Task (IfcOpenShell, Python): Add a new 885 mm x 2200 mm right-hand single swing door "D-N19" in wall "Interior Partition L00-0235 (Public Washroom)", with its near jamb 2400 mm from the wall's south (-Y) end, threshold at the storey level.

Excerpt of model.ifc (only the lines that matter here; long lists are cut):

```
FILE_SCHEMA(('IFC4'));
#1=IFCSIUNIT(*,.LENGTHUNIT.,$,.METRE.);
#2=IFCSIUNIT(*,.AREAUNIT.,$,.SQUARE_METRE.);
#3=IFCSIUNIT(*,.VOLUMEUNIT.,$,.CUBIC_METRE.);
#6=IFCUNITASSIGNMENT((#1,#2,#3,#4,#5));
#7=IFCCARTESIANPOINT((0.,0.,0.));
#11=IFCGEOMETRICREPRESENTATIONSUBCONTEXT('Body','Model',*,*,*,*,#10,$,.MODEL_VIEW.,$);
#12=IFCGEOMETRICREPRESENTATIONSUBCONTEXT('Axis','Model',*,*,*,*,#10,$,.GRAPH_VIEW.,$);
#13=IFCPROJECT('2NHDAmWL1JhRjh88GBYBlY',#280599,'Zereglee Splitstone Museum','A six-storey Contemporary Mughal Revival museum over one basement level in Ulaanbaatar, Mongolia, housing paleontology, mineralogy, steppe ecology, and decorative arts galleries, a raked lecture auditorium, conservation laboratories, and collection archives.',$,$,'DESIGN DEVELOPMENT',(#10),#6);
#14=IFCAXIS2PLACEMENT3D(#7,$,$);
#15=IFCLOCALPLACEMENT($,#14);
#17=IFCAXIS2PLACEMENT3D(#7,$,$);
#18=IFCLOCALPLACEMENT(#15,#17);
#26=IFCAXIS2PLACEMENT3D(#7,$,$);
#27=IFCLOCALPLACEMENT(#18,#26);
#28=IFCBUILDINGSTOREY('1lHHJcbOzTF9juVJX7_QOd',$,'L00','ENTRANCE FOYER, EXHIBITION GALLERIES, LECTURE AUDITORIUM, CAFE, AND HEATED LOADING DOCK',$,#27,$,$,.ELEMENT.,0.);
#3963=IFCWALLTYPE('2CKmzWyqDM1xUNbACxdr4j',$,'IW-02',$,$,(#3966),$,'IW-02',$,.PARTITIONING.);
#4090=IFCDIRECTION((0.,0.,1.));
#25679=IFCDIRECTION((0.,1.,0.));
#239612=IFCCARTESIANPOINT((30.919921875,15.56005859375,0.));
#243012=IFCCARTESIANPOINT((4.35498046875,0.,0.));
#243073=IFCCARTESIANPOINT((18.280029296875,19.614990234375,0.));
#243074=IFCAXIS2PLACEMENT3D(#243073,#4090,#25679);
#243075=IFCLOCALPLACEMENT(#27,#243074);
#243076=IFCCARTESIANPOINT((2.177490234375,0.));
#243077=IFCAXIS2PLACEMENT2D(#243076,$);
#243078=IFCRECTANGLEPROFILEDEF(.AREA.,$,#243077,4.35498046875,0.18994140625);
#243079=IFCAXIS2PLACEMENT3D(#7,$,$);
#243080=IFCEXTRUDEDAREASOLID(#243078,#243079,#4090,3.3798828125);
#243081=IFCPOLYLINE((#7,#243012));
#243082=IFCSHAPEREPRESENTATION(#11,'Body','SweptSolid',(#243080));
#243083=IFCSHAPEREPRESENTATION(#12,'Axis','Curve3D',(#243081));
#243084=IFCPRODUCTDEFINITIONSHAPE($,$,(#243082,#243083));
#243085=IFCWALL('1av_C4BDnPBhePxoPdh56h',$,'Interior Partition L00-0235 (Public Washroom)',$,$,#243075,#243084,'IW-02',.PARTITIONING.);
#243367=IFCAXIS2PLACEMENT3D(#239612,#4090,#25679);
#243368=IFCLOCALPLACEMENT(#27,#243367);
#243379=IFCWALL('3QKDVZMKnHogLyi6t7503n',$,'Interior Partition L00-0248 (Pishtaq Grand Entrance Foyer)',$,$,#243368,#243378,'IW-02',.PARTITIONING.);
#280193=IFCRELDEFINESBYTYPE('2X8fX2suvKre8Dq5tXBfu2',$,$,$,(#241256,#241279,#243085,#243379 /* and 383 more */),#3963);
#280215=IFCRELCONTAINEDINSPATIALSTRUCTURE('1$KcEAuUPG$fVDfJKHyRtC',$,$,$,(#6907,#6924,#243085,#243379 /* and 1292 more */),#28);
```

```python
import numpy as np
import ifcopenshell
import ifcopenshell.api.feature
import ifcopenshell.api.geometry
import ifcopenshell.api.root
import ifcopenshell.api.spatial
import ifcopenshell.geom
import ifcopenshell.util.element
import ifcopenshell.util.placement
import ifcopenshell.util.representation
import ifcopenshell.util.shape
import ifcopenshell.util.unit

model = ifcopenshell.open("model.ifc")
unit_scale = ifcopenshell.util.unit.calculate_unit_scale(model)
settings = ifcopenshell.geom.settings()


def volume(element):
    """Net volume in cubic metres, openings subtracted."""
    shape = ifcopenshell.geom.create_shape(settings, element)
    return ifcopenshell.util.shape.get_volume(shape.geometry)


wall = model.by_guid("1av_C4BDnPBhePxoPdh56h")
storey = ifcopenshell.util.element.get_container(wall, ifc_class="IfcBuildingStorey")
context = ifcopenshell.util.representation.get_context(model, "Model", "Body", "MODEL_VIEW")
before = volume(wall)

width, height, from_end, sill = 0.885, 2.2, 2.4, 0.0  # metres

# The wall runs along its own X axis, and the end named is its -X end.
wall_shape = ifcopenshell.geom.create_shape(settings, wall)
x, y, z = ifcopenshell.util.shape.get_vertices(wall_shape.geometry).T
start = x.min() + from_end
face, thickness = float(y.min()), float(y.max() - y.min())
wall_matrix = ifcopenshell.util.placement.get_local_placement(wall.ObjectPlacement)
level = ifcopenshell.util.placement.get_local_placement(storey.ObjectPlacement)[2, 3]


def in_wall(x, y):
    """Placement at x, y metres in the wall's axes, at sill height."""
    matrix = wall_matrix.copy()
    matrix[:, 3] = wall_matrix @ np.array([x / unit_scale, y / unit_scale, 0.0, 1.0])
    matrix[2, 3] = level + sill / unit_scale
    return matrix


# Opening: a box that overshoots both wall faces by 50 mm.
opening = ifcopenshell.api.root.create_entity(model, ifc_class="IfcOpeningElement", predefined_type="OPENING")
box = ifcopenshell.api.geometry.add_wall_representation(
    model, context=context, length=width, height=height, thickness=thickness + 0.1
)
ifcopenshell.api.geometry.assign_representation(model, product=opening, representation=box)
ifcopenshell.api.geometry.edit_object_placement(model, product=opening, matrix=in_wall(start, face - 0.05), is_si=False)
ifcopenshell.api.feature.add_feature(model, feature=opening, element=wall)

door = ifcopenshell.api.root.create_entity(model, ifc_class="IfcDoor", name="D-N19", predefined_type="DOOR")
door.OverallWidth, door.OverallHeight = width / unit_scale, height / unit_scale
door.OperationType = "SINGLE_SWING_RIGHT"
body = ifcopenshell.api.geometry.add_door_representation(
    model,
    context=context,
    overall_width=door.OverallWidth,
    overall_height=door.OverallHeight,
    operation_type="SINGLE_SWING_RIGHT",
    lining_properties={"LiningDepth": thickness / unit_scale, "ThresholdDepth": thickness / unit_scale},
)
ifcopenshell.api.geometry.assign_representation(model, product=door, representation=body)
ifcopenshell.api.spatial.assign_container(model, products=[door], relating_structure=storey)
ifcopenshell.api.feature.add_filling(model, opening=opening, element=door)

# The lining spans the wall, so the door starts at the wall face.
ifcopenshell.api.geometry.edit_object_placement(model, product=door, matrix=in_wall(start, face), is_si=False)

after = volume(wall)

print(f"wall volume {before:.3f} -> {after:.3f} m3")

model.write("model_updated.ifc")
```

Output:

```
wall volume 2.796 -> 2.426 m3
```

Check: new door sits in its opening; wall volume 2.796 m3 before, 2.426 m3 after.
